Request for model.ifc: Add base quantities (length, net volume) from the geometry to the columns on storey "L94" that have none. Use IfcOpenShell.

First a look at what the model holds.

```python
import ifcopenshell
import ifcopenshell.util.element
import ifcopenshell.util.unit

model = ifcopenshell.open("model.ifc")
print(model.schema)
for unit_type in ("LENGTHUNIT", "AREAUNIT", "VOLUMEUNIT"):
    print(unit_type, ifcopenshell.util.unit.calculate_unit_scale(model, unit_type))
storey = next(s for s in model.by_type("IfcBuildingStorey") if s.Name == "L94")
columns = [e for e in ifcopenshell.util.element.get_decomposition(storey) if e.is_a("IfcColumn")]
for e in sorted(columns, key=lambda e: e.id()):
    print(e.id(), e.is_a(), e.Name, list(ifcopenshell.util.element.get_psets(e, qtos_only=True)), sep=" | ")
```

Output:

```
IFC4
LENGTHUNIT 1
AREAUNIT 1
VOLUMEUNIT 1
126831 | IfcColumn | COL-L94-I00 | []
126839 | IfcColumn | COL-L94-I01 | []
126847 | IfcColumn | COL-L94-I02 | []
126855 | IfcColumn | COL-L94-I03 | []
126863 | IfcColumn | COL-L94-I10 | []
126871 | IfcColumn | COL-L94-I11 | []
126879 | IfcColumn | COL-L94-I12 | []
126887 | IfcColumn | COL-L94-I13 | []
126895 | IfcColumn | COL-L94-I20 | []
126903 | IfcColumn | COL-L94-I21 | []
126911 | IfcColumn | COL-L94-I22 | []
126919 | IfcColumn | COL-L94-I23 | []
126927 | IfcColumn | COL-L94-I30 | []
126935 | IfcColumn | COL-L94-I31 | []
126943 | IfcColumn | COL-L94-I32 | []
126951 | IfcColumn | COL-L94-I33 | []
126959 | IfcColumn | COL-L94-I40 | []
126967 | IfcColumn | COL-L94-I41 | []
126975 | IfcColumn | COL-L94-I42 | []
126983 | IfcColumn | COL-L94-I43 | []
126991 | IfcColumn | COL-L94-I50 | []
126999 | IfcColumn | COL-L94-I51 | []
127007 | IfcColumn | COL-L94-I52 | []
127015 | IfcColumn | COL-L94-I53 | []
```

```python
import ifcopenshell
import ifcopenshell.api.pset
import ifcopenshell.geom
import ifcopenshell.util.element
import ifcopenshell.util.shape
import ifcopenshell.util.unit

model = ifcopenshell.open("model.ifc")
unit_scale = ifcopenshell.util.unit.calculate_unit_scale(model)
volume_scale = ifcopenshell.util.unit.calculate_unit_scale(model, "VOLUMEUNIT")
settings = ifcopenshell.geom.settings()

storey = next(s for s in model.by_type("IfcBuildingStorey") if s.Name == "L94")
columns = [e for e in ifcopenshell.util.element.get_decomposition(storey) if e.is_a("IfcColumn")]

for e in sorted(columns, key=lambda e: e.id()):
    if ifcopenshell.util.element.get_psets(e, qtos_only=True, should_inherit=False):
        continue
    # Geometry comes back in metres, in the element's own axes.
    shape = ifcopenshell.geom.create_shape(settings, e)
    values = {
        "Length": ifcopenshell.util.shape.get_z(shape.geometry) / unit_scale,
        "NetVolume": ifcopenshell.util.shape.get_volume(shape.geometry) / volume_scale,
    }
    qto = ifcopenshell.api.pset.add_qto(model, product=e, name="Qto_ColumnBaseQuantities")
    ifcopenshell.api.pset.edit_qto(model, qto=qto, properties=values)
    print(e.id(), {k: round(v, 3) for k, v in values.items()})

model.write("model_v2.ifc")
```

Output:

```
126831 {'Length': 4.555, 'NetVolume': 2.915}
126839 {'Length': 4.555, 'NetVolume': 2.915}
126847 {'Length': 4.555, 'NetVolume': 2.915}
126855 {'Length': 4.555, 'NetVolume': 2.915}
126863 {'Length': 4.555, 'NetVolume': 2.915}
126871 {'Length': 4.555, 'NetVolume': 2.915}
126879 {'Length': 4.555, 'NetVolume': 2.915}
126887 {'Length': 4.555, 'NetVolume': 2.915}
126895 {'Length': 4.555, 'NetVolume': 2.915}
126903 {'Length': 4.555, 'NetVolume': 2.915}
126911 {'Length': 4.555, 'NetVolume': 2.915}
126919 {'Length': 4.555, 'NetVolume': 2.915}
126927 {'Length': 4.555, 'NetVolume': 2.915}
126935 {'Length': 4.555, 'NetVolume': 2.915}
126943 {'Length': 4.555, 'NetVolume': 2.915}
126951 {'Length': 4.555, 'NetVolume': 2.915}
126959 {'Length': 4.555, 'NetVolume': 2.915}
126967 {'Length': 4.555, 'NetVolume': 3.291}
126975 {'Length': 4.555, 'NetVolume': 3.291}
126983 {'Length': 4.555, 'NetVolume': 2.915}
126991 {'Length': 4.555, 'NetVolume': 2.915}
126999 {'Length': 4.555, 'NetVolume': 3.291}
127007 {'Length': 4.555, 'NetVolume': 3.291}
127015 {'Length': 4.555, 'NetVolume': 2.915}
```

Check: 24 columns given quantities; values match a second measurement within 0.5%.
